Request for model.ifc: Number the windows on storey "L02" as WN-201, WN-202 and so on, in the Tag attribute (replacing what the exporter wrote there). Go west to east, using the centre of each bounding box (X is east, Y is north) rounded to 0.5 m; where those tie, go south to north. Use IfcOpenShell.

First a look at what the model holds.

```python
import ifcopenshell
import ifcopenshell.util.element
import ifcopenshell.util.placement

model = ifcopenshell.open("model.ifc")
print(model.schema)
storey = next(s for s in model.by_type("IfcBuildingStorey") if s.Name == "L02")
windows = [e for e in ifcopenshell.util.element.get_decomposition(storey) if e.is_a("IfcWindow")]
for e in sorted(windows, key=lambda e: e.id()):
    origin = ifcopenshell.util.placement.get_local_placement(e.ObjectPlacement)[:3, 3]
    print(e.id(), e.Tag, e.Name, origin.round(2) + 0.0, sep=" | ")
```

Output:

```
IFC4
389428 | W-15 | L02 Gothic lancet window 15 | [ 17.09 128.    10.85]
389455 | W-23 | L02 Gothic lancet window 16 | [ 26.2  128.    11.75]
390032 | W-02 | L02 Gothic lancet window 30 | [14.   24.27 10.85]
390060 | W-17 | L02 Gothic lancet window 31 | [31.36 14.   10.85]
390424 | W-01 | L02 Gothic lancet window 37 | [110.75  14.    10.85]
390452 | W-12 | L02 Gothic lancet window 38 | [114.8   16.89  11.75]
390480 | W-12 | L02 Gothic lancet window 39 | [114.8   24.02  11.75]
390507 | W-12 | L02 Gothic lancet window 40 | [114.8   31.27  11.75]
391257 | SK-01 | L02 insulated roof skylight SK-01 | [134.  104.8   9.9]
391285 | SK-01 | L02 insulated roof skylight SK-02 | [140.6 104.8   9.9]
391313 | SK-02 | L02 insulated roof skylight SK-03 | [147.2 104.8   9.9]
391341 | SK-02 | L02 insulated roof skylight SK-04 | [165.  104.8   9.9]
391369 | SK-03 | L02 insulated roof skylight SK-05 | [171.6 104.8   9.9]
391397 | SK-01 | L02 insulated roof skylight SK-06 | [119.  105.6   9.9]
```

```python
import ifcopenshell
import ifcopenshell.geom
import ifcopenshell.util.element
import ifcopenshell.util.shape

model = ifcopenshell.open("model.ifc")
settings = ifcopenshell.geom.settings()
settings.set("use-world-coords", True)


def centre(element):
    shape = ifcopenshell.geom.create_shape(settings, element)
    return ifcopenshell.util.shape.get_bbox_centroid(shape.geometry)


storey = next(s for s in model.by_type("IfcBuildingStorey") if s.Name == "L02")
windows = [e for e in ifcopenshell.util.element.get_decomposition(storey) if e.is_a("IfcWindow")]

# Insertion points can sit at a corner or the storey origin, so sort by the geometry (in metres).
centres = {e: centre(e) for e in windows}
windows.sort(key=lambda e: (round(centres[e][0] / 0.5), centres[e][1]))

for i, e in enumerate(windows, start=1):
    number = f"WN-2{i:02d}"
    e.Tag = number
    print(e.id(), number)

model.write("model_rev.ifc")
```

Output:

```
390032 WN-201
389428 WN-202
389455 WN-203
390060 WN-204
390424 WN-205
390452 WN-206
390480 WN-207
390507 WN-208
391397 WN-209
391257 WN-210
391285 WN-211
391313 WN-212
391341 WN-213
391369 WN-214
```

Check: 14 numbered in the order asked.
